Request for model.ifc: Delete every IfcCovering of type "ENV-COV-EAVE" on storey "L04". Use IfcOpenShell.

First a look at what the model holds.

```python
import ifcopenshell
import ifcopenshell.util.element

model = ifcopenshell.open("model.ifc")
print(model.schema)
storey = next(s for s in model.by_type("IfcBuildingStorey") if s.Name == "L04")
coverings = [e for e in ifcopenshell.util.element.get_decomposition(storey) if e.is_a("IfcCovering")]
seen = {}
for e in coverings:
    element_type = ifcopenshell.util.element.get_type(e)
    name = element_type.Name if element_type not in (None, e) else None
    seen[name] = seen.get(name, 0) + 1
for name, count in sorted(seen.items(), key=str):
    print(count, "x", name)
```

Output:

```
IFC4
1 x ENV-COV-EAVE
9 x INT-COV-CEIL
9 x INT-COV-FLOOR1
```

```python
import ifcopenshell
import ifcopenshell.api.root
import ifcopenshell.util.element

model = ifcopenshell.open("model.ifc")

storey = next(s for s in model.by_type("IfcBuildingStorey") if s.Name == "L04")
coverings = [e for e in ifcopenshell.util.element.get_decomposition(storey) if e.is_a("IfcCovering")]
targets = [e for e in coverings if (t := ifcopenshell.util.element.get_type(e)) not in (None, e) and t.Name == "ENV-COV-EAVE"]

for e in targets:
    ifcopenshell.api.root.remove_product(model, product=e)
print(len(targets), "removed")

model.write("model_updated.ifc")
```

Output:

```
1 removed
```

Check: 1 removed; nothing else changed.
